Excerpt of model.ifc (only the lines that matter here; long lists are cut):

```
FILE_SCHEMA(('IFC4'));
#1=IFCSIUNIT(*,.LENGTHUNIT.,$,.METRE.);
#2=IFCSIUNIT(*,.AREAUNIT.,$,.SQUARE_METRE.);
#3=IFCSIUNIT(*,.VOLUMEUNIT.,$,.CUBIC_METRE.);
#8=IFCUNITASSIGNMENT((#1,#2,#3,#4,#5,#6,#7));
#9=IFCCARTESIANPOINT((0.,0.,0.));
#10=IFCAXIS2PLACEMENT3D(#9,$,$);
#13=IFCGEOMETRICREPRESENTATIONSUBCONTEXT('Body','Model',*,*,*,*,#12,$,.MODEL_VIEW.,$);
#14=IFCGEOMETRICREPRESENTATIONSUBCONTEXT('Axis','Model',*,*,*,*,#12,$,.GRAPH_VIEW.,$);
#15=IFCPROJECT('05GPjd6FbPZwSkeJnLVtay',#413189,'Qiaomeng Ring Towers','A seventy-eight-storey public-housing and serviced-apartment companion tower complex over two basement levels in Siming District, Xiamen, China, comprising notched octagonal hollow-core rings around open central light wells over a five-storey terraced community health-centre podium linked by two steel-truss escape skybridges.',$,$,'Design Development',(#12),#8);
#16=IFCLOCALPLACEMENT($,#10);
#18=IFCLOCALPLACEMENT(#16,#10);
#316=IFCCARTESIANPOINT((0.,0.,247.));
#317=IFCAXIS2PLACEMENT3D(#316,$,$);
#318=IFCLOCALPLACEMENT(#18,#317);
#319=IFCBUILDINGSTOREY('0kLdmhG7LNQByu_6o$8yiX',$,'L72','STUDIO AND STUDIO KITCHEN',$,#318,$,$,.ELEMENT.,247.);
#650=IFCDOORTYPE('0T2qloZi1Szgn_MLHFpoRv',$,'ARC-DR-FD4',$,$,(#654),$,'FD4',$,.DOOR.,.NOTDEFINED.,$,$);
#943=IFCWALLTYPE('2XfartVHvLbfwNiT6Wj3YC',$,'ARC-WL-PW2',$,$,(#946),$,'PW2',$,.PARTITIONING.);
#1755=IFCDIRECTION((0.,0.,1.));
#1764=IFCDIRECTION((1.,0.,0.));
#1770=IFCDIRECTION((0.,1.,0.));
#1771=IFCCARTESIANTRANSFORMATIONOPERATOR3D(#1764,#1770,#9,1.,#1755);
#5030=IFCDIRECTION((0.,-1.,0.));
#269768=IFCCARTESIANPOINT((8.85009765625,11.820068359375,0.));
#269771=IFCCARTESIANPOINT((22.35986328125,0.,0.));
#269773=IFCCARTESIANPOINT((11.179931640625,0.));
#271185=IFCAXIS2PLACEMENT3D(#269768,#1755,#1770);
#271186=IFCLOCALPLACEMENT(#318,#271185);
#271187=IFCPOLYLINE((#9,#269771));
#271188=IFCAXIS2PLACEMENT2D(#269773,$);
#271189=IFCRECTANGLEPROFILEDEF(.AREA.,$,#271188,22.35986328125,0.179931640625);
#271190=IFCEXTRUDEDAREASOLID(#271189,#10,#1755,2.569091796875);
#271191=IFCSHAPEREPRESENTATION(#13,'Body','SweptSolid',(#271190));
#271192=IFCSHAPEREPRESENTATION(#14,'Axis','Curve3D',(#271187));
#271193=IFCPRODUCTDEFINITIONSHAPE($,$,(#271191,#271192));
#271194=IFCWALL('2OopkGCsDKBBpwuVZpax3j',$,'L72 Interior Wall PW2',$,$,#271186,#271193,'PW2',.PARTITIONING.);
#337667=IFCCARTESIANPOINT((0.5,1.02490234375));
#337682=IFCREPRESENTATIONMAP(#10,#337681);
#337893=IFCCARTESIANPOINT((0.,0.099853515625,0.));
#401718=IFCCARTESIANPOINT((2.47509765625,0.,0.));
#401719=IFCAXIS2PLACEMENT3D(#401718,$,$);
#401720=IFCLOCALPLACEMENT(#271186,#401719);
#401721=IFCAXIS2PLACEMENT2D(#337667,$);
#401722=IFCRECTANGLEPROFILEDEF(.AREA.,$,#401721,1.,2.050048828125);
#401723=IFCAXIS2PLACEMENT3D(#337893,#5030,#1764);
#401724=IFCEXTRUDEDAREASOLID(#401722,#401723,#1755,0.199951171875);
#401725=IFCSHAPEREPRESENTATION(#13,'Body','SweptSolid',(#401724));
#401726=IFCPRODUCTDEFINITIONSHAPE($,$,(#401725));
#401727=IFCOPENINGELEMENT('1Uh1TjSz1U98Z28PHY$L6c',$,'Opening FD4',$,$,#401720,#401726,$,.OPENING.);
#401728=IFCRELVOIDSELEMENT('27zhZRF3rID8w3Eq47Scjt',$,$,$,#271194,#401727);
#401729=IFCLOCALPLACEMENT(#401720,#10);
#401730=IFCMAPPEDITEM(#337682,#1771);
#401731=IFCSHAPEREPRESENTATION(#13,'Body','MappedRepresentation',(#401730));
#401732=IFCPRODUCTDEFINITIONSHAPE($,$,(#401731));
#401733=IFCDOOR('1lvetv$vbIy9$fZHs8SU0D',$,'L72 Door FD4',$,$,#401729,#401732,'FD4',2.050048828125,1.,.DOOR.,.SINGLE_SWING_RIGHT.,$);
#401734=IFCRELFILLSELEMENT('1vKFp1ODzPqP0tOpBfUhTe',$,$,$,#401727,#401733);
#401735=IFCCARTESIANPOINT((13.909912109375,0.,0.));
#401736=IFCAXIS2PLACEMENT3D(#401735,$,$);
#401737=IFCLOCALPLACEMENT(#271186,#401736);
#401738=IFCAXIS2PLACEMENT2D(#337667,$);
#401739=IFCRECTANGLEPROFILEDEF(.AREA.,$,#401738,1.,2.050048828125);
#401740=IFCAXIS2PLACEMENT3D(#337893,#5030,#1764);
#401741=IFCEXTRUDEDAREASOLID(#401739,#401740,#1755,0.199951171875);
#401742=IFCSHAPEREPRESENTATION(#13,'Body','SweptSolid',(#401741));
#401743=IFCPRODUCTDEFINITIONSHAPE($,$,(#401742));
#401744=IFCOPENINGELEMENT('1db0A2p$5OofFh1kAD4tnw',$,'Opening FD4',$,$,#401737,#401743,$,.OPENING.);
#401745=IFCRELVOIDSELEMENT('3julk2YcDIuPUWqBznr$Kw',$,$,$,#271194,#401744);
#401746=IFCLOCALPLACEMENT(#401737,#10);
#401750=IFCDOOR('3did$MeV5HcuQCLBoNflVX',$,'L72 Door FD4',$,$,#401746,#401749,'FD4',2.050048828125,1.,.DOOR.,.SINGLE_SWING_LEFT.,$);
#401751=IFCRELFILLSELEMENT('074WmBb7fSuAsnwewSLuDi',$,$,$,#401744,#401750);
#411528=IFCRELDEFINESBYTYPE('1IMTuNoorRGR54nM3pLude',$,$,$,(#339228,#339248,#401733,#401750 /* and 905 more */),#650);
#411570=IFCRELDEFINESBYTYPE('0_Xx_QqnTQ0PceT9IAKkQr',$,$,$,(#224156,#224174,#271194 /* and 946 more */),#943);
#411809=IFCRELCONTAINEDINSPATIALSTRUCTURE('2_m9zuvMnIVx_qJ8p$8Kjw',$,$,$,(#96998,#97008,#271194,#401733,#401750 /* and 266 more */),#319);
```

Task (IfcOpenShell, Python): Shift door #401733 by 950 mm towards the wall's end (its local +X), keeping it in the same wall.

```python
import ifcopenshell
import ifcopenshell.api.geometry
import ifcopenshell.util.placement
import ifcopenshell.util.unit

model = ifcopenshell.open("model.ifc")
unit_scale = ifcopenshell.util.unit.calculate_unit_scale(model)

door = model.by_guid("1lvetv$vbIy9$fZHs8SU0D")
opening = door.FillsVoids[0].RelatingOpeningElement
wall = opening.VoidsElements[0].RelatingBuildingElement

wall_matrix = ifcopenshell.util.placement.get_local_placement(wall.ObjectPlacement)
shift = wall_matrix[:3, 0] * 0.95 / unit_scale
before = ifcopenshell.util.placement.get_local_placement(door.ObjectPlacement)[:3, 3].copy()

# The door is placed relative to its opening, so it follows when the opening moves.
matrix = ifcopenshell.util.placement.get_local_placement(opening.ObjectPlacement)
matrix[:3, 3] += shift
ifcopenshell.api.geometry.edit_object_placement(
    model, product=opening, matrix=matrix, is_si=False, should_transform_children=True
)

after = ifcopenshell.util.placement.get_local_placement(door.ObjectPlacement)[:3, 3]
print("door moved by", (after - before).round(3) + 0.0)

model.write("model_updated.ifc")
```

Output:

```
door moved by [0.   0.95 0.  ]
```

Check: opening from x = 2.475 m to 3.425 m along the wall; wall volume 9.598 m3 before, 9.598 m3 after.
